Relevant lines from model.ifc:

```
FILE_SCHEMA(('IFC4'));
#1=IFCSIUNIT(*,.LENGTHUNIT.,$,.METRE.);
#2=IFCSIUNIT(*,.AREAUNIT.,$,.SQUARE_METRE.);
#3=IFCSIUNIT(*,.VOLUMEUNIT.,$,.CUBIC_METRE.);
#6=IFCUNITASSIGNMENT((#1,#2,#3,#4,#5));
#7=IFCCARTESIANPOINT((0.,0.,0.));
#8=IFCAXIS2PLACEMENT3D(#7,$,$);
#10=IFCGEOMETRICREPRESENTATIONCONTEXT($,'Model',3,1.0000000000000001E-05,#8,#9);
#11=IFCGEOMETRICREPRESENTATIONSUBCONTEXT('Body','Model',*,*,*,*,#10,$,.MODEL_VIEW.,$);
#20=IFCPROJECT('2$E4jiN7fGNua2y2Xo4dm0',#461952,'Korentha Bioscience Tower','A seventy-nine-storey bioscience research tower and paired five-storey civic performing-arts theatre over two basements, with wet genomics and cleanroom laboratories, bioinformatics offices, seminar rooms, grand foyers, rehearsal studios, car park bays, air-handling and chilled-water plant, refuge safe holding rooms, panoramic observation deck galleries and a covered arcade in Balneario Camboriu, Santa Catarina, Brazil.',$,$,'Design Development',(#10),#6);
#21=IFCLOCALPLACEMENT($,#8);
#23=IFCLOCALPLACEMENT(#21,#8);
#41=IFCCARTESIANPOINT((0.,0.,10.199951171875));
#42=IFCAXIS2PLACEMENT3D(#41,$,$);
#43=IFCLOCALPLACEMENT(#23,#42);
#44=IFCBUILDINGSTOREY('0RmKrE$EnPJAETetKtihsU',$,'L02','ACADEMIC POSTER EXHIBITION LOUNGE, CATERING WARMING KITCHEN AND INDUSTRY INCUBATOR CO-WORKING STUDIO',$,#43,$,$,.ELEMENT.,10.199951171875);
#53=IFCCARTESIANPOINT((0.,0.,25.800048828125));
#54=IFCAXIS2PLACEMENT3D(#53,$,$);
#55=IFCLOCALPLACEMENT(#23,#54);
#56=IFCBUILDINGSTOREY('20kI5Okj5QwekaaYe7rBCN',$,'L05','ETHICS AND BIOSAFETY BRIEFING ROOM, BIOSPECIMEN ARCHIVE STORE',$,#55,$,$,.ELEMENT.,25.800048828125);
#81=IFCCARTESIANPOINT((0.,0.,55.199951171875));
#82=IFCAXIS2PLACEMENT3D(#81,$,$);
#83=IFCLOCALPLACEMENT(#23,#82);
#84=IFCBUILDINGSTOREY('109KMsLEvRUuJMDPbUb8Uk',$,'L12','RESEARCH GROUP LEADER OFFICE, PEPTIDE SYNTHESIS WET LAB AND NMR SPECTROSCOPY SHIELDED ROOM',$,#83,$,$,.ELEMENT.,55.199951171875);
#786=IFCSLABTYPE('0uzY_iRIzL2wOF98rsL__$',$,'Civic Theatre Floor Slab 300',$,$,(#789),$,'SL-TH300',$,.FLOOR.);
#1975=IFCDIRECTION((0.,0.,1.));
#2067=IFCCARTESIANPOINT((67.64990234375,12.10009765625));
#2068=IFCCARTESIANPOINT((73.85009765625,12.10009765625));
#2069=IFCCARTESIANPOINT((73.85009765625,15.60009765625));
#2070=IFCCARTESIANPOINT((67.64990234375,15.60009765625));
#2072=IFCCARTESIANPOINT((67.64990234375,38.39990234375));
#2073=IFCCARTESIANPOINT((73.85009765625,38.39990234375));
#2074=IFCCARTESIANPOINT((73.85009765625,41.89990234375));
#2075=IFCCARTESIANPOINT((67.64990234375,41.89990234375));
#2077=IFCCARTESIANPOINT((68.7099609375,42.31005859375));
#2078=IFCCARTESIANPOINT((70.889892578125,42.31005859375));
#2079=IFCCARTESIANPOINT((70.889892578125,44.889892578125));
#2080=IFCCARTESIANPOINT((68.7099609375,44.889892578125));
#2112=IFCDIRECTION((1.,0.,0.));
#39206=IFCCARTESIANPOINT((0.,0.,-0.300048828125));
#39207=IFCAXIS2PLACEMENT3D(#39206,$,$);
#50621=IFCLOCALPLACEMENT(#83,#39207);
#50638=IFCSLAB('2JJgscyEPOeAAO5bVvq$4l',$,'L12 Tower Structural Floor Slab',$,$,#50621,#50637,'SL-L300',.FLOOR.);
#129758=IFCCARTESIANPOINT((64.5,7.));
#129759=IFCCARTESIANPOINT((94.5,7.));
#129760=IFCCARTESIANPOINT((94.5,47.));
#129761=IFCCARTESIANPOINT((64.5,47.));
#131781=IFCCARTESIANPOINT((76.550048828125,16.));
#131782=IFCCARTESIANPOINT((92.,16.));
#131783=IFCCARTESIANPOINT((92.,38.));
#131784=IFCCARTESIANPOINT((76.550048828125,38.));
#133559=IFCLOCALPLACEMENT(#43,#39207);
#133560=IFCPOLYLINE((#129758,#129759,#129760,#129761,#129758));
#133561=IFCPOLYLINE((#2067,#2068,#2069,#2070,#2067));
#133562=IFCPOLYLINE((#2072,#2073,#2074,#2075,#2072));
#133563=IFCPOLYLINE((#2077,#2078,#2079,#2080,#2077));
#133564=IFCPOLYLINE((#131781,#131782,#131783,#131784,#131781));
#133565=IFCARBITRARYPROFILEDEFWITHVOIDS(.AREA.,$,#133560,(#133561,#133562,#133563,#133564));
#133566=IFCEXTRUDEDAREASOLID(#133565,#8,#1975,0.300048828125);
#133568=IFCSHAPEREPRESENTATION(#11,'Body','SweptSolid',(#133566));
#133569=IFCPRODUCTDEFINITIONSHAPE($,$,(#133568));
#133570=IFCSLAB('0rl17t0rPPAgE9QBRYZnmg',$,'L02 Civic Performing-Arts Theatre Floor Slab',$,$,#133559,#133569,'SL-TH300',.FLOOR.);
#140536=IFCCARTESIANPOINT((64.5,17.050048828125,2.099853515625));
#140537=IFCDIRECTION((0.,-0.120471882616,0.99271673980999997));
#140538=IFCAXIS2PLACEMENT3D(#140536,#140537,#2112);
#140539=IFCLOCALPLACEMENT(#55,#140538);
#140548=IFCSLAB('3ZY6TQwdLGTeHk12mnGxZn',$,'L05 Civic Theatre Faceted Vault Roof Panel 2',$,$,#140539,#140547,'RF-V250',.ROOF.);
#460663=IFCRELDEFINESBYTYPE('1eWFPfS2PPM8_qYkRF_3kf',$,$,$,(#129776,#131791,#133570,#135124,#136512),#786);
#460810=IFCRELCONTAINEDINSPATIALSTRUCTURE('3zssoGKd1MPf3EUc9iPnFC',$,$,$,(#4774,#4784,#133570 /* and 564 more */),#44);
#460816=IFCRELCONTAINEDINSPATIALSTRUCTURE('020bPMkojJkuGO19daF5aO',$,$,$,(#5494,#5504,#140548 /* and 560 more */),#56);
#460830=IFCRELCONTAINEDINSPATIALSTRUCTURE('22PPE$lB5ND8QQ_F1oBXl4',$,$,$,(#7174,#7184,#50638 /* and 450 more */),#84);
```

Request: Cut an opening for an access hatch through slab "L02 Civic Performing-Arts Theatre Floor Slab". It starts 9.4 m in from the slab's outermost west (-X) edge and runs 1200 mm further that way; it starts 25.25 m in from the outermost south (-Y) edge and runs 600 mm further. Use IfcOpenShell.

```python
import numpy as np
import ifcopenshell
import ifcopenshell.api.feature
import ifcopenshell.api.geometry
import ifcopenshell.api.root
import ifcopenshell.geom
import ifcopenshell.util.placement
import ifcopenshell.util.representation
import ifcopenshell.util.shape
import ifcopenshell.util.unit

model = ifcopenshell.open("model.ifc")
unit_scale = ifcopenshell.util.unit.calculate_unit_scale(model)
settings = ifcopenshell.geom.settings()


def volume(element):
    """Net volume in cubic metres, openings subtracted."""
    shape = ifcopenshell.geom.create_shape(settings, element)
    return ifcopenshell.util.shape.get_volume(shape.geometry)


slab = model.by_guid("0rl17t0rPPAgE9QBRYZnmg")
before = volume(slab)

# Extent in the slab's own axes, in metres. The edges named are its -X and -Y sides.
slab_shape = ifcopenshell.geom.create_shape(settings, slab)
vertices = ifcopenshell.util.shape.get_vertices(slab_shape.geometry)
x_min, y_min, bottom = vertices.min(axis=0)
top = vertices[:, 2].max()

opening = ifcopenshell.api.root.create_entity(model, ifc_class="IfcOpeningElement", name="Access hatch opening", predefined_type="OPENING")
context = ifcopenshell.util.representation.get_context(model, "Model", "Body", "MODEL_VIEW")
width, depth = 1.2, 0.6
outline = [(0.0, 0.0), (width, 0.0), (width, depth), (0.0, depth), (0.0, 0.0)]
# Overshoot both faces by 50 mm so the cut is clean.
shape = ifcopenshell.api.geometry.add_slab_representation(
    model, context=context, depth=top - bottom + 0.1, polyline=outline
)
ifcopenshell.api.geometry.assign_representation(model, product=opening, representation=shape)

matrix = ifcopenshell.util.placement.get_local_placement(slab.ObjectPlacement)
matrix[:, 3] = matrix @ np.append(np.array([x_min + 9.4, y_min + 25.25, bottom - 0.05]) / unit_scale, 1.0)
ifcopenshell.api.geometry.edit_object_placement(model, product=opening, matrix=matrix, is_si=False)
ifcopenshell.api.feature.add_feature(model, feature=opening, element=slab)

after = volume(slab)

print(f"slab volume {before:.3f} -> {after:.3f} m3")

model.write("model_updated.ifc")
```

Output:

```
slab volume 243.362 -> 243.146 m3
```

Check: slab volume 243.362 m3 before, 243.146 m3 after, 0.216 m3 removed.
